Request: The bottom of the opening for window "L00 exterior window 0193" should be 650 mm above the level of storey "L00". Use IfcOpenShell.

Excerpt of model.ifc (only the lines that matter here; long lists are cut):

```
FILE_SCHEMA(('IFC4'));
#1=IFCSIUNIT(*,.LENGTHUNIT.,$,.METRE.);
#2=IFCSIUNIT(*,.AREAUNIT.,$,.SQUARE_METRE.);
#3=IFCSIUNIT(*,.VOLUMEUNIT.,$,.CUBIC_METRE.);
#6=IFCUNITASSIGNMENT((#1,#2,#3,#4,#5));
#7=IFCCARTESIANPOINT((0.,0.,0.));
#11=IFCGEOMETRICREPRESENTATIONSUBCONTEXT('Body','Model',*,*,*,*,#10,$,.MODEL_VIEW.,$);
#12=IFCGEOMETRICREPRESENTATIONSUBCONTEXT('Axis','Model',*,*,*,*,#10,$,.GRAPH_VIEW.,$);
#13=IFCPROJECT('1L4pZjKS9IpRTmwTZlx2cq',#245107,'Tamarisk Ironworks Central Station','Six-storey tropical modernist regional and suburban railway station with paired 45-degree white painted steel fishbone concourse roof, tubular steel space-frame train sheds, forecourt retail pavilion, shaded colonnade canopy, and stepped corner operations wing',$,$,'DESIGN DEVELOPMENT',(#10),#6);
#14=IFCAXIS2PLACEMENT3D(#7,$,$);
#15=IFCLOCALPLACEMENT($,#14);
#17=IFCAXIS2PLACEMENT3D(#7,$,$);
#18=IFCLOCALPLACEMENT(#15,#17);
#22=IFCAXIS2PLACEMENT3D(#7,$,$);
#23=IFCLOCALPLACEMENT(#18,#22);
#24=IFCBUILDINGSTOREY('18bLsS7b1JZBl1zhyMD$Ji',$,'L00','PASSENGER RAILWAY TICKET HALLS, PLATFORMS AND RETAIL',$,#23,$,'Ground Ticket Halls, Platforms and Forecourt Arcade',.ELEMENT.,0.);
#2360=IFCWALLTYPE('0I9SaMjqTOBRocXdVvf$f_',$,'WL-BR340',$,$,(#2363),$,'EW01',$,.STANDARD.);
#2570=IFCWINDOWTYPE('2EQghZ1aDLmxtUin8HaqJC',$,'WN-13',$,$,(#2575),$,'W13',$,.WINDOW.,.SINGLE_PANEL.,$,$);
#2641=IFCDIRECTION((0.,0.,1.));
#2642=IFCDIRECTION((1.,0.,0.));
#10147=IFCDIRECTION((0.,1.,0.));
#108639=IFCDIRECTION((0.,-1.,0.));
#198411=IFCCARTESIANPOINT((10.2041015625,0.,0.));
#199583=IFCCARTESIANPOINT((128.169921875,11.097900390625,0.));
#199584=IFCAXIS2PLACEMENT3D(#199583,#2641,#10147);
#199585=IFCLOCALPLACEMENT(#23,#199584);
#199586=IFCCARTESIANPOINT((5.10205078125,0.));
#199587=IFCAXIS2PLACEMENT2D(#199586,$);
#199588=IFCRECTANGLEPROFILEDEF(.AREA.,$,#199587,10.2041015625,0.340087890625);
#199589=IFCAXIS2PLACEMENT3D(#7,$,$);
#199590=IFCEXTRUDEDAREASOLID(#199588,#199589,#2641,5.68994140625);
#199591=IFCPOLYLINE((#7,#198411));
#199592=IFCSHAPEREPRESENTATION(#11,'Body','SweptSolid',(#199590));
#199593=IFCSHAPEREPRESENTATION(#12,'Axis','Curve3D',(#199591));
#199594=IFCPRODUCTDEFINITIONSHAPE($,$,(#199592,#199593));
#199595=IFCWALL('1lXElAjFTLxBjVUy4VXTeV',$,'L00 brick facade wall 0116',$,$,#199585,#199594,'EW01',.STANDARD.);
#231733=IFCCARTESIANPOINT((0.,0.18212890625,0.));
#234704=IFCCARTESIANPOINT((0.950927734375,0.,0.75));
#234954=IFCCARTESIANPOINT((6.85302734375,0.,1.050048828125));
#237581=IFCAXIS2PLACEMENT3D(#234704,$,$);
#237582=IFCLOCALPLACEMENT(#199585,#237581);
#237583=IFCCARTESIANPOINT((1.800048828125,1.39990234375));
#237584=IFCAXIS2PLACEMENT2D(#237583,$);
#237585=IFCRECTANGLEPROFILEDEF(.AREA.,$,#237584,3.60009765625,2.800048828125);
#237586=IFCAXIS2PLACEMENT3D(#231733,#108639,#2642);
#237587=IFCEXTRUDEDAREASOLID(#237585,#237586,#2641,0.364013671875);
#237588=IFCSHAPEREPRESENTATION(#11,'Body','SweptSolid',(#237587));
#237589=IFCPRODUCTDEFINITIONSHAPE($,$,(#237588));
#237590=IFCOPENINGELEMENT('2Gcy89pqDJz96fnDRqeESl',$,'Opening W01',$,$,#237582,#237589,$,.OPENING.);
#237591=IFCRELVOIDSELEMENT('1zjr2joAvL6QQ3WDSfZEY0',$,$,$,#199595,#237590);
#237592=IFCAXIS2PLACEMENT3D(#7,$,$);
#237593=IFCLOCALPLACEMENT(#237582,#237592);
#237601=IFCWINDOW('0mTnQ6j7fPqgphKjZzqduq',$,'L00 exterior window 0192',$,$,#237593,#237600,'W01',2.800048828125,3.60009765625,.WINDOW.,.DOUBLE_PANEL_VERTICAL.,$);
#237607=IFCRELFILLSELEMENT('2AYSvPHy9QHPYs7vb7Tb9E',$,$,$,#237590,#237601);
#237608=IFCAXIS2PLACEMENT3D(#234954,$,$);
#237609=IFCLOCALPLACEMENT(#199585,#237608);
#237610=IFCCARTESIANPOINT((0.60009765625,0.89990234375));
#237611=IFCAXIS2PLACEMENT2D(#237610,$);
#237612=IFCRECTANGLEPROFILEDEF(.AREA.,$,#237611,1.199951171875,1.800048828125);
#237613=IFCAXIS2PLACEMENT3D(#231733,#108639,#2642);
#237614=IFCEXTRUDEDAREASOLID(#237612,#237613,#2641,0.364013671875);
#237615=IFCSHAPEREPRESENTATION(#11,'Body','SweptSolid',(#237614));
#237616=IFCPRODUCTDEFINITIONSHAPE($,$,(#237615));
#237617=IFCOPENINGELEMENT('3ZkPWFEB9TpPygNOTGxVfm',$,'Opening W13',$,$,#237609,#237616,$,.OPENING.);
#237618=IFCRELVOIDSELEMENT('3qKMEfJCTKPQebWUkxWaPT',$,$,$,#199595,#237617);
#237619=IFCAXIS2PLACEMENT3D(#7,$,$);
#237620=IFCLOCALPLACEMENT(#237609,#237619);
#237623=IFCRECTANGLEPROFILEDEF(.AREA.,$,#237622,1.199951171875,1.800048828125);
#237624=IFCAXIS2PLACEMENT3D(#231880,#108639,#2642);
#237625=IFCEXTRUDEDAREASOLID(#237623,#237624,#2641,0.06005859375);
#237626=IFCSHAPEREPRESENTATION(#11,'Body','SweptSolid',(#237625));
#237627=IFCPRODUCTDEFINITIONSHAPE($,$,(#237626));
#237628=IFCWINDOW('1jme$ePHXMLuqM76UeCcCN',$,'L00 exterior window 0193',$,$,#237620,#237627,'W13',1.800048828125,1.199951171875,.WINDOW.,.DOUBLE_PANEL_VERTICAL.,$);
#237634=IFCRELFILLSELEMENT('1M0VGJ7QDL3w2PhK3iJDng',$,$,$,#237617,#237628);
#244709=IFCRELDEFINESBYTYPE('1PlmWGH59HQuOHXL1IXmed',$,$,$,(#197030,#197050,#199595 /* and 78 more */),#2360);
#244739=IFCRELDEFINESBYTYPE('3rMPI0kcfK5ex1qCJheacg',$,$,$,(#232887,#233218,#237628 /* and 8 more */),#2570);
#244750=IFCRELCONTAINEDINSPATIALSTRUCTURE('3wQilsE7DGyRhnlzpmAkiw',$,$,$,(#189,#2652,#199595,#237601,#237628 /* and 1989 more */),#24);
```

```python
import numpy as np
import ifcopenshell
import ifcopenshell.api.geometry
import ifcopenshell.geom
import ifcopenshell.util.element
import ifcopenshell.util.placement
import ifcopenshell.util.shape
import ifcopenshell.util.unit

model = ifcopenshell.open("model.ifc")
unit_scale = ifcopenshell.util.unit.calculate_unit_scale(model)

window = model.by_guid("1jme$ePHXMLuqM76UeCcCN")
opening = window.FillsVoids[0].RelatingOpeningElement
storey = ifcopenshell.util.element.get_container(window, ifc_class="IfcBuildingStorey")
level = ifcopenshell.util.placement.get_local_placement(storey.ObjectPlacement)[2, 3]

# The opening's origin need not be at the sill, so measure its lowest point.
shape = ifcopenshell.geom.create_shape(ifcopenshell.geom.settings(), opening)
bottom = ifcopenshell.util.shape.get_shape_bottom_elevation(shape, shape.geometry) / unit_scale
dz = level + 0.65 / unit_scale - bottom

shift = np.array([0.0, 0.0, dz])
# The window is placed relative to its opening, so it follows when the opening moves.
matrix = ifcopenshell.util.placement.get_local_placement(opening.ObjectPlacement)
matrix[:3, 3] += shift
ifcopenshell.api.geometry.edit_object_placement(
    model, product=opening, matrix=matrix, is_si=False, should_transform_children=True
)

print(f"moved by {dz * unit_scale:+.3f} m")

model.write("model_v2.ifc")
```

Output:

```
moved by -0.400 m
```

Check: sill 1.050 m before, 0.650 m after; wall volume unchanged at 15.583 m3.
